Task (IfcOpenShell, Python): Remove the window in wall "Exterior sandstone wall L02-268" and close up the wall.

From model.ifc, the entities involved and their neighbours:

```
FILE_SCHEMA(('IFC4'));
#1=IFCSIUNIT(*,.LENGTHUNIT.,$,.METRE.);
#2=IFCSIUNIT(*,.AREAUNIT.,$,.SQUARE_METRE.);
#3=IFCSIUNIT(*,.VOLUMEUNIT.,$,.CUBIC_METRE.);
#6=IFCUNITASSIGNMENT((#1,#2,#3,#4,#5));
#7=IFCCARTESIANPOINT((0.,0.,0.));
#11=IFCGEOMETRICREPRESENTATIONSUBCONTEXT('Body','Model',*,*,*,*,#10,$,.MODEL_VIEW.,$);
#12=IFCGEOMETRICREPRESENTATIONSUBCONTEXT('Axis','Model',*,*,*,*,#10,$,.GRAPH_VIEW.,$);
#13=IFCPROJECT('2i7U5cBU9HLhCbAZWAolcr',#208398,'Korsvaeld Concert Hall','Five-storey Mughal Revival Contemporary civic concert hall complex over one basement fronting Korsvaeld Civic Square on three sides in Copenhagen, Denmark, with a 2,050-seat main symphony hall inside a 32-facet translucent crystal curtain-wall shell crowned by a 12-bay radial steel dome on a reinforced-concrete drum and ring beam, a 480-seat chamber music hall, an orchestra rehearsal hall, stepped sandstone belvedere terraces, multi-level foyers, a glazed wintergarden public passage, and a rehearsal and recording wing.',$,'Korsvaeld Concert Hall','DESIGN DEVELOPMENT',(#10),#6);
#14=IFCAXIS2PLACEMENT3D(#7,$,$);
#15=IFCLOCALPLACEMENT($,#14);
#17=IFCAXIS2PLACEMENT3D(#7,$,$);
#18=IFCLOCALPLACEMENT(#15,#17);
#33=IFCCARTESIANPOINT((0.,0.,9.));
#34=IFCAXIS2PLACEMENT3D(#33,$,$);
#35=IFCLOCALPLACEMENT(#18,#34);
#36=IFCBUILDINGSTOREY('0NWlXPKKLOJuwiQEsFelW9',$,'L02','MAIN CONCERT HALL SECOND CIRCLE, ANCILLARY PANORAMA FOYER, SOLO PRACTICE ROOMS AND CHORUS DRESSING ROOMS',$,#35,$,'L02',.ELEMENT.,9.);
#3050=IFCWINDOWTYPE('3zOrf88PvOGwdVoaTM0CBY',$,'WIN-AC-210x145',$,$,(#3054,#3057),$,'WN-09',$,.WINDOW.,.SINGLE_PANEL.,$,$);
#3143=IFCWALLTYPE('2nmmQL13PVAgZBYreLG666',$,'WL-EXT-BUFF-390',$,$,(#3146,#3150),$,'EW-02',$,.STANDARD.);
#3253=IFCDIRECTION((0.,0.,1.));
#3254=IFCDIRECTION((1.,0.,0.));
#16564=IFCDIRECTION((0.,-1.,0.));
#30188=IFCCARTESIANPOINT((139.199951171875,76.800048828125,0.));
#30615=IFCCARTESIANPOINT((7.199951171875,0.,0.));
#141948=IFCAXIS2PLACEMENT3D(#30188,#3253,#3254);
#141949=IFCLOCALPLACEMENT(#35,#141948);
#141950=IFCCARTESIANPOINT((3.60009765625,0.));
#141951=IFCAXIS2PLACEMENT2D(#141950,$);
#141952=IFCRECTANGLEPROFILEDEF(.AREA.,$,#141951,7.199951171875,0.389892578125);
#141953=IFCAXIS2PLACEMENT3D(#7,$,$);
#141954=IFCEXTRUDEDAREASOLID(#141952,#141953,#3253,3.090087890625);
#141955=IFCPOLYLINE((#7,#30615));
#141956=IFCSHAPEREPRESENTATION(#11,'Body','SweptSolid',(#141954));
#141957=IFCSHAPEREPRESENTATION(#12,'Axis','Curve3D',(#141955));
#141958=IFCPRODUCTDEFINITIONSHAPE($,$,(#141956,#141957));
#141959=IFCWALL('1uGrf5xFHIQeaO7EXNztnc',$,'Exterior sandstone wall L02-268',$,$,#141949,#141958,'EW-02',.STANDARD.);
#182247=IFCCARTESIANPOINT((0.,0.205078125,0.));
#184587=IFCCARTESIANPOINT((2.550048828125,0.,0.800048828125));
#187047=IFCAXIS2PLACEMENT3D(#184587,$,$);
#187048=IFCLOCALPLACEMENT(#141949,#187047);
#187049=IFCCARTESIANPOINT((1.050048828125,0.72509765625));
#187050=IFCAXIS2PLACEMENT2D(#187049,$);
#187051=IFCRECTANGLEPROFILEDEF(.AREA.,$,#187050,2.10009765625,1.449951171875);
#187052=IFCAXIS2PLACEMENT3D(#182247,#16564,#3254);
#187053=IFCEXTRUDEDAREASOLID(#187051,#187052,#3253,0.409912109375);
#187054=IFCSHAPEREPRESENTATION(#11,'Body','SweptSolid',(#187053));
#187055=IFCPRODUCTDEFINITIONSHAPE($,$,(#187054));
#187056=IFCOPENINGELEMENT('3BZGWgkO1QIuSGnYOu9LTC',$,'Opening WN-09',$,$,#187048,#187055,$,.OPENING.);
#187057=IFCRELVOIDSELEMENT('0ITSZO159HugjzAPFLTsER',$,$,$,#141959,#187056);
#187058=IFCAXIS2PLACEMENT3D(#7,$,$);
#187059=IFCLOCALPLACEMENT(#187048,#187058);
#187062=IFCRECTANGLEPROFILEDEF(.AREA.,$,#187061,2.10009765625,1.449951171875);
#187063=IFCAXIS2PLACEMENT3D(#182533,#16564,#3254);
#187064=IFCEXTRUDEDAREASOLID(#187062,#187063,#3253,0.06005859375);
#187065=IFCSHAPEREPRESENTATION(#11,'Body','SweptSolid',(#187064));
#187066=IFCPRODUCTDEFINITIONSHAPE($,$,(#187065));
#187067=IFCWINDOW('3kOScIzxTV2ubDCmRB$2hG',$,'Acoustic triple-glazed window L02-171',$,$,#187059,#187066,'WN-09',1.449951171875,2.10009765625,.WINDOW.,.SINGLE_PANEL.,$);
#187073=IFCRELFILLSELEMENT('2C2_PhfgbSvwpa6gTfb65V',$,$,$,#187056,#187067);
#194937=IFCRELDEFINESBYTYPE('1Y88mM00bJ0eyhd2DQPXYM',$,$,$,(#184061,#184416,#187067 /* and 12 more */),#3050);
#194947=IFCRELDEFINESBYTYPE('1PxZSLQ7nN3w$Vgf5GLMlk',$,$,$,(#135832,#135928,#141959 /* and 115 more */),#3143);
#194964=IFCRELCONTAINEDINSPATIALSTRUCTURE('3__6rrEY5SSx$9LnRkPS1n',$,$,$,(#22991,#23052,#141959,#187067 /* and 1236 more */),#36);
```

```python
import ifcopenshell
import ifcopenshell.api.feature
import ifcopenshell.api.root
import ifcopenshell.geom
import ifcopenshell.util.shape

model = ifcopenshell.open("model.ifc")
settings = ifcopenshell.geom.settings()


def volume(element):
    """Net volume in cubic metres, openings subtracted."""
    shape = ifcopenshell.geom.create_shape(settings, element)
    return ifcopenshell.util.shape.get_volume(shape.geometry)


window = model.by_guid("3kOScIzxTV2ubDCmRB$2hG")
opening = window.FillsVoids[0].RelatingOpeningElement
wall = opening.VoidsElements[0].RelatingBuildingElement
before = volume(wall)

ifcopenshell.api.root.remove_product(model, product=window)
ifcopenshell.api.feature.remove_feature(model, feature=opening)

after = volume(wall)

print(f"wall volume {before:.3f} -> {after:.3f} m3")

model.write("model_edited.ifc")
```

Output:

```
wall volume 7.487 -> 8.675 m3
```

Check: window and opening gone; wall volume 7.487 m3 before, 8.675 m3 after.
